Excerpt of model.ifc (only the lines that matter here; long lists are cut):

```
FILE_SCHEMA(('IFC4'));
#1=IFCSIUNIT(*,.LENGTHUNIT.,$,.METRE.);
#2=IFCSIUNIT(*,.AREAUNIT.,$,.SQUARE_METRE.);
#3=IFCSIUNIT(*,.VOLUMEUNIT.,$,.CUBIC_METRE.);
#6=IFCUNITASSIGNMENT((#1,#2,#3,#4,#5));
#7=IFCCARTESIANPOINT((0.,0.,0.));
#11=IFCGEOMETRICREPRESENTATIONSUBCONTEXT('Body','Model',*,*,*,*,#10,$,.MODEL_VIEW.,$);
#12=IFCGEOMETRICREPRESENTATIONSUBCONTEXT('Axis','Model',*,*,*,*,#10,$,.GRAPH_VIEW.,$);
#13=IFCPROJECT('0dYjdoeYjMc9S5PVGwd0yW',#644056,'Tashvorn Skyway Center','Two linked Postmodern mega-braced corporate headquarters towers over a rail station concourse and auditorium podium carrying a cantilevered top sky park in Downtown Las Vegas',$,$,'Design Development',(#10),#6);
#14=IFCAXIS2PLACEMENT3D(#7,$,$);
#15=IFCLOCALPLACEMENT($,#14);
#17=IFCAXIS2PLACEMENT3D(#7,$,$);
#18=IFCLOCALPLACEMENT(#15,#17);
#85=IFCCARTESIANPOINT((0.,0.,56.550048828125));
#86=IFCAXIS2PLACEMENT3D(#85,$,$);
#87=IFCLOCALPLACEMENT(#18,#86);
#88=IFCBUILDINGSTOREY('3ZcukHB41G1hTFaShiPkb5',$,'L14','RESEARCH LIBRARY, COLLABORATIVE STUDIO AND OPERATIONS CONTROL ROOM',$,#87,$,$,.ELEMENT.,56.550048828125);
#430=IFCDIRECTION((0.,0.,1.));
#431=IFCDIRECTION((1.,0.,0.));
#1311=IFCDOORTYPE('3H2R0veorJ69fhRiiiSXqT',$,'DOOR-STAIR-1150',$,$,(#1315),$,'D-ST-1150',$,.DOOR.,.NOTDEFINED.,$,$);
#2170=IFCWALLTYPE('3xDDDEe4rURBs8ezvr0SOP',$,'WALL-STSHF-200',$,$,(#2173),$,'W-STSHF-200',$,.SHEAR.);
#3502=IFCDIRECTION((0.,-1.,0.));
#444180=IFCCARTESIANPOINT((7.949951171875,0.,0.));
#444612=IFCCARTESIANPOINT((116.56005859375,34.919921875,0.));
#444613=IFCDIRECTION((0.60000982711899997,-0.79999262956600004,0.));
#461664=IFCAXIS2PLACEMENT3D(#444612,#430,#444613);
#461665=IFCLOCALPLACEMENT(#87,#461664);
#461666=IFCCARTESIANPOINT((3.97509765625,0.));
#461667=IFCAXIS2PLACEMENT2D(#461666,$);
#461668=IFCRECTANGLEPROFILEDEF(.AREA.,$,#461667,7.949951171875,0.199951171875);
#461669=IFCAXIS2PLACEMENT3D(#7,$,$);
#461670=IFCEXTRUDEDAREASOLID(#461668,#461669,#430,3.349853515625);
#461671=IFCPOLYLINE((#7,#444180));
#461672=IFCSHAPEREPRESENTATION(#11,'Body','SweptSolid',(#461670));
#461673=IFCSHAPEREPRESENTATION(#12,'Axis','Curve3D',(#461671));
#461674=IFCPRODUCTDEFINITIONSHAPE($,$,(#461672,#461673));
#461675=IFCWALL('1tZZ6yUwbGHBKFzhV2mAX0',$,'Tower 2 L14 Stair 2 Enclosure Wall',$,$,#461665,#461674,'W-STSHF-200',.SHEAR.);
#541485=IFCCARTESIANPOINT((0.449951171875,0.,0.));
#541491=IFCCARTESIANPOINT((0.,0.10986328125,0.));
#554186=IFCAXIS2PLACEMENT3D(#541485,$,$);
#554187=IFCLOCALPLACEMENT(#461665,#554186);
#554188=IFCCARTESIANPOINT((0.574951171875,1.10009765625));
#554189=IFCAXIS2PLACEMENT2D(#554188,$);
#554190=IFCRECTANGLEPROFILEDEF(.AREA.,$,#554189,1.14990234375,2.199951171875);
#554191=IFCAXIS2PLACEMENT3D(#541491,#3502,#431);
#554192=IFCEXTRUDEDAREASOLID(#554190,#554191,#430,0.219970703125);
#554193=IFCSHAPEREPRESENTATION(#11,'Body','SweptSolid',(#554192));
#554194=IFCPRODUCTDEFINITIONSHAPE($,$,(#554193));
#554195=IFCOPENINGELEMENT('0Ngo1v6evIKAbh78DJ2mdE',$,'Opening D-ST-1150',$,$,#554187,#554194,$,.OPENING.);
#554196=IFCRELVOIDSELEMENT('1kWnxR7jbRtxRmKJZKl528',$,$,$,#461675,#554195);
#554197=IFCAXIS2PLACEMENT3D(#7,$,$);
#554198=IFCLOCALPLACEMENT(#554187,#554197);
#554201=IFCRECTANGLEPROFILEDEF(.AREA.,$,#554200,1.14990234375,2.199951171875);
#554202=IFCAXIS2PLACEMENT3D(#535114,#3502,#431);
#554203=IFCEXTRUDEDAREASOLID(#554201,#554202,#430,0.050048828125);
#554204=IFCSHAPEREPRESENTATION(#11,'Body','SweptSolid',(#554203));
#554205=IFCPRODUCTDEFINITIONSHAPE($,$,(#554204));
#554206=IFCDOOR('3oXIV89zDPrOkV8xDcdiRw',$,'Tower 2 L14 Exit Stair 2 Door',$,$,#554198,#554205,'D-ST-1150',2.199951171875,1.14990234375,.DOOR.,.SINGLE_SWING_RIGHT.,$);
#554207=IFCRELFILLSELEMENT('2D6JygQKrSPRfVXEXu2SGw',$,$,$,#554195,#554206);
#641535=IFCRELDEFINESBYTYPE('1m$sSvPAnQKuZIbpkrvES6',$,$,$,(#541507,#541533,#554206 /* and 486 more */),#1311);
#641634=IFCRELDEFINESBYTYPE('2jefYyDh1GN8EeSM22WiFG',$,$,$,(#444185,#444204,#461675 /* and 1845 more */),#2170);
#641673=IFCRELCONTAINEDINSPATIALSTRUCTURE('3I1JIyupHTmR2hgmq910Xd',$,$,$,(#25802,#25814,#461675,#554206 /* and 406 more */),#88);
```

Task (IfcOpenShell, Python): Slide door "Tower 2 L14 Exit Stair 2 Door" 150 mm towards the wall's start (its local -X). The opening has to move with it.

```python
import ifcopenshell
import ifcopenshell.api.geometry
import ifcopenshell.util.placement
import ifcopenshell.util.unit

model = ifcopenshell.open("model.ifc")
unit_scale = ifcopenshell.util.unit.calculate_unit_scale(model)

door = model.by_id(554206)
opening = door.FillsVoids[0].RelatingOpeningElement
wall = opening.VoidsElements[0].RelatingBuildingElement

wall_matrix = ifcopenshell.util.placement.get_local_placement(wall.ObjectPlacement)
shift = wall_matrix[:3, 0] * -0.15 / unit_scale
before = ifcopenshell.util.placement.get_local_placement(door.ObjectPlacement)[:3, 3].copy()

# The door is placed relative to its opening, so it follows when the opening moves.
matrix = ifcopenshell.util.placement.get_local_placement(opening.ObjectPlacement)
matrix[:3, 3] += shift
ifcopenshell.api.geometry.edit_object_placement(
    model, product=opening, matrix=matrix, is_si=False, should_transform_children=True
)

after = ifcopenshell.util.placement.get_local_placement(door.ObjectPlacement)[:3, 3]
print("door moved by", (after - before).round(3) + 0.0)

model.write("model-out.ifc")
```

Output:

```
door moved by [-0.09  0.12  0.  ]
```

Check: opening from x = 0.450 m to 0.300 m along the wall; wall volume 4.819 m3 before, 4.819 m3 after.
